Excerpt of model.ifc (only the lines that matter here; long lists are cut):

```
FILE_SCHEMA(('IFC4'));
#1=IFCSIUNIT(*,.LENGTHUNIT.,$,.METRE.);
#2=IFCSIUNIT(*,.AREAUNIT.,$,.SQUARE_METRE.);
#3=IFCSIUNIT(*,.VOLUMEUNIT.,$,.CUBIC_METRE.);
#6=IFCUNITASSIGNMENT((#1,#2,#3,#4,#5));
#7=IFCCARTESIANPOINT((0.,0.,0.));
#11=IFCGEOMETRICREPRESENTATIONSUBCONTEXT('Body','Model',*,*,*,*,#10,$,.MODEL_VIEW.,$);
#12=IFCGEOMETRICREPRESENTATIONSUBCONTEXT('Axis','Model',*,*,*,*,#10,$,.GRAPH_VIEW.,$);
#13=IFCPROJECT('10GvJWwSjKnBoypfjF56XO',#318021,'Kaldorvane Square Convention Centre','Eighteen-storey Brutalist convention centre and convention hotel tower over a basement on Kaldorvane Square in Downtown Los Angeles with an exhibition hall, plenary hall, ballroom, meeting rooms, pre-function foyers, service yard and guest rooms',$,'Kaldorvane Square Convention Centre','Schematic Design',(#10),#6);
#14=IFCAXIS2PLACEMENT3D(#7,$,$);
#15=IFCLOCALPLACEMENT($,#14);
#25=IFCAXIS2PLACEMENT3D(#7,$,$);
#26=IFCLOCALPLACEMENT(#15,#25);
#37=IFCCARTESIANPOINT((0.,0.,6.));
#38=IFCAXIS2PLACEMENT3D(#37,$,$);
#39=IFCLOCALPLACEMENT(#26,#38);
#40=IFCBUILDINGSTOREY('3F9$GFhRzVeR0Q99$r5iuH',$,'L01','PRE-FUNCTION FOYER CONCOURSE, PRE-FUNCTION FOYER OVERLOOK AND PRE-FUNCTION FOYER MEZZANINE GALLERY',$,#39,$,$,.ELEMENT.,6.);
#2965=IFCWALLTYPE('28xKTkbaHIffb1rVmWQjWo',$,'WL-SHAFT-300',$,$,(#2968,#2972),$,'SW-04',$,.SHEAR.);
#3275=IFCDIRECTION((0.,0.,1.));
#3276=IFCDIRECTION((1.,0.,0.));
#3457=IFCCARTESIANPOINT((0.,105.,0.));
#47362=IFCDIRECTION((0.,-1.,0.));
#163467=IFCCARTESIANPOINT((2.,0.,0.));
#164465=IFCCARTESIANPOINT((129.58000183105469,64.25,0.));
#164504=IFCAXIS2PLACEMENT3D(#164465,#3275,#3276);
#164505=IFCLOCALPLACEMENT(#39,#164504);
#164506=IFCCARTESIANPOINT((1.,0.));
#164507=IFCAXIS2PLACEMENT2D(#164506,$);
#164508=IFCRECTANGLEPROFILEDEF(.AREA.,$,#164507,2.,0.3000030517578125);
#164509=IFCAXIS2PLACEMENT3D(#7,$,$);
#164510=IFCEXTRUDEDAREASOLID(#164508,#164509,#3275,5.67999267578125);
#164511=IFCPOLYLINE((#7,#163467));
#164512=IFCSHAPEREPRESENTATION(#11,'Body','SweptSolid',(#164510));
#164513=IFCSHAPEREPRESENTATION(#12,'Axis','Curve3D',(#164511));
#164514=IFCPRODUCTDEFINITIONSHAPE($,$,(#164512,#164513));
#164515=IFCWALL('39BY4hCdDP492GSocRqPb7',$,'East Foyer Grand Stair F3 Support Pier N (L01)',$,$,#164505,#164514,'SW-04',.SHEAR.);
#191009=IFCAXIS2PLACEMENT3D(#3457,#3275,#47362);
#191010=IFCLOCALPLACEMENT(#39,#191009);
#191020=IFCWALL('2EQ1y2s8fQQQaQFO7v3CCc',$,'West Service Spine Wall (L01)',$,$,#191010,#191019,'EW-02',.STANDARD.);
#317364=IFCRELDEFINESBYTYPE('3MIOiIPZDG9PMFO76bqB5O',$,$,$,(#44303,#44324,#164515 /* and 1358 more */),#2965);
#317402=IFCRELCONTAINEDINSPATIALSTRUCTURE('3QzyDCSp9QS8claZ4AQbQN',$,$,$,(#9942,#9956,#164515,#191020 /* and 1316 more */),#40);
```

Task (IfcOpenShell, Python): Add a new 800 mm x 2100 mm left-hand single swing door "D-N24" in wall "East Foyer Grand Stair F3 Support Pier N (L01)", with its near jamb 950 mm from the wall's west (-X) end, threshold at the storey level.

```python
import numpy as np
import ifcopenshell
import ifcopenshell.api.feature
import ifcopenshell.api.geometry
import ifcopenshell.api.root
import ifcopenshell.api.spatial
import ifcopenshell.geom
import ifcopenshell.util.element
import ifcopenshell.util.placement
import ifcopenshell.util.representation
import ifcopenshell.util.shape
import ifcopenshell.util.unit

model = ifcopenshell.open("model.ifc")
unit_scale = ifcopenshell.util.unit.calculate_unit_scale(model)
settings = ifcopenshell.geom.settings()


def volume(element):
    """Net volume in cubic metres, openings subtracted."""
    shape = ifcopenshell.geom.create_shape(settings, element)
    return ifcopenshell.util.shape.get_volume(shape.geometry)


wall = model.by_id(164515)
storey = ifcopenshell.util.element.get_container(wall, ifc_class="IfcBuildingStorey")
context = ifcopenshell.util.representation.get_context(model, "Model", "Body", "MODEL_VIEW")
before = volume(wall)

width, height, from_end, sill = 0.8, 2.1, 0.95, 0.0  # metres

# The wall runs along its own X axis, and the end named is its -X end.
wall_shape = ifcopenshell.geom.create_shape(settings, wall)
x, y, z = ifcopenshell.util.shape.get_vertices(wall_shape.geometry).T
start = x.min() + from_end
face, thickness = float(y.min()), float(y.max() - y.min())
wall_matrix = ifcopenshell.util.placement.get_local_placement(wall.ObjectPlacement)
level = ifcopenshell.util.placement.get_local_placement(storey.ObjectPlacement)[2, 3]


def in_wall(x, y):
    """Placement at x, y metres in the wall's axes, at sill height."""
    matrix = wall_matrix.copy()
    matrix[:, 3] = wall_matrix @ np.array([x / unit_scale, y / unit_scale, 0.0, 1.0])
    matrix[2, 3] = level + sill / unit_scale
    return matrix


# Opening: a box that overshoots both wall faces by 50 mm.
opening = ifcopenshell.api.root.create_entity(model, ifc_class="IfcOpeningElement", predefined_type="OPENING")
box = ifcopenshell.api.geometry.add_wall_representation(
    model, context=context, length=width, height=height, thickness=thickness + 0.1
)
ifcopenshell.api.geometry.assign_representation(model, product=opening, representation=box)
ifcopenshell.api.geometry.edit_object_placement(model, product=opening, matrix=in_wall(start, face - 0.05), is_si=False)
ifcopenshell.api.feature.add_feature(model, feature=opening, element=wall)

door = ifcopenshell.api.root.create_entity(model, ifc_class="IfcDoor", name="D-N24", predefined_type="DOOR")
door.OverallWidth, door.OverallHeight = width / unit_scale, height / unit_scale
door.OperationType = "SINGLE_SWING_LEFT"
body = ifcopenshell.api.geometry.add_door_representation(
    model,
    context=context,
    overall_width=door.OverallWidth,
    overall_height=door.OverallHeight,
    operation_type="SINGLE_SWING_LEFT",
    lining_properties={"LiningDepth": thickness / unit_scale, "ThresholdDepth": thickness / unit_scale},
)
ifcopenshell.api.geometry.assign_representation(model, product=door, representation=body)
ifcopenshell.api.spatial.assign_container(model, products=[door], relating_structure=storey)
ifcopenshell.api.feature.add_filling(model, opening=opening, element=door)

# The lining spans the wall, so the door starts at the wall face.
ifcopenshell.api.geometry.edit_object_placement(model, product=door, matrix=in_wall(start, face), is_si=False)

after = volume(wall)

print(f"wall volume {before:.3f} -> {after:.3f} m3")

model.write("model_edited.ifc")
```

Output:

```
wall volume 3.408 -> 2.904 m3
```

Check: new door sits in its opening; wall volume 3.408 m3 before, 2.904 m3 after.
